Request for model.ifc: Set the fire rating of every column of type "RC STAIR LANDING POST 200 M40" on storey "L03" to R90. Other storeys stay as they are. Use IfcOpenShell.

First a look at what the model holds.

```python
import ifcopenshell
import ifcopenshell.util.element

model = ifcopenshell.open("model.ifc")
print(model.schema)
storey = next(s for s in model.by_type("IfcBuildingStorey") if s.Name == "L03")
columns = [e for e in ifcopenshell.util.element.get_decomposition(storey) if e.is_a("IfcColumn")]
seen = {}
for e in columns:
    element_type = ifcopenshell.util.element.get_type(e)
    key = (element_type.Name if element_type != e and element_type else None, ifcopenshell.util.element.get_pset(e, "Pset_ColumnCommon", "FireRating"))
    seen[key] = seen.get(key, 0) + 1
for (name, value), count in sorted(seen.items(), key=str):
    print(count, "x", name, "|", value)
```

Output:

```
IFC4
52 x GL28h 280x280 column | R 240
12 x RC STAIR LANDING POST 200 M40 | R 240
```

```python
import ifcopenshell
import ifcopenshell.api.pset
import ifcopenshell.util.element

model = ifcopenshell.open("model.ifc")

storey = next(s for s in model.by_type("IfcBuildingStorey") if s.Name == "L03")
columns = [e for e in ifcopenshell.util.element.get_decomposition(storey) if e.is_a("IfcColumn")]

count = 0
for e in columns:
    element_type = ifcopenshell.util.element.get_type(e)
    if element_type in (None, e) or element_type.Name != "RC STAIR LANDING POST 200 M40":
        continue
    # add_pset returns the element's existing set when there is one.
    pset = ifcopenshell.api.pset.add_pset(model, product=e, name="Pset_ColumnCommon")
    ifcopenshell.api.pset.edit_pset(model, pset=pset, properties={"FireRating": "R90"})
    count += 1

print(count, "columns updated")

model.write("model_edited.ifc")
```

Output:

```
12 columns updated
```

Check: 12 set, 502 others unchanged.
